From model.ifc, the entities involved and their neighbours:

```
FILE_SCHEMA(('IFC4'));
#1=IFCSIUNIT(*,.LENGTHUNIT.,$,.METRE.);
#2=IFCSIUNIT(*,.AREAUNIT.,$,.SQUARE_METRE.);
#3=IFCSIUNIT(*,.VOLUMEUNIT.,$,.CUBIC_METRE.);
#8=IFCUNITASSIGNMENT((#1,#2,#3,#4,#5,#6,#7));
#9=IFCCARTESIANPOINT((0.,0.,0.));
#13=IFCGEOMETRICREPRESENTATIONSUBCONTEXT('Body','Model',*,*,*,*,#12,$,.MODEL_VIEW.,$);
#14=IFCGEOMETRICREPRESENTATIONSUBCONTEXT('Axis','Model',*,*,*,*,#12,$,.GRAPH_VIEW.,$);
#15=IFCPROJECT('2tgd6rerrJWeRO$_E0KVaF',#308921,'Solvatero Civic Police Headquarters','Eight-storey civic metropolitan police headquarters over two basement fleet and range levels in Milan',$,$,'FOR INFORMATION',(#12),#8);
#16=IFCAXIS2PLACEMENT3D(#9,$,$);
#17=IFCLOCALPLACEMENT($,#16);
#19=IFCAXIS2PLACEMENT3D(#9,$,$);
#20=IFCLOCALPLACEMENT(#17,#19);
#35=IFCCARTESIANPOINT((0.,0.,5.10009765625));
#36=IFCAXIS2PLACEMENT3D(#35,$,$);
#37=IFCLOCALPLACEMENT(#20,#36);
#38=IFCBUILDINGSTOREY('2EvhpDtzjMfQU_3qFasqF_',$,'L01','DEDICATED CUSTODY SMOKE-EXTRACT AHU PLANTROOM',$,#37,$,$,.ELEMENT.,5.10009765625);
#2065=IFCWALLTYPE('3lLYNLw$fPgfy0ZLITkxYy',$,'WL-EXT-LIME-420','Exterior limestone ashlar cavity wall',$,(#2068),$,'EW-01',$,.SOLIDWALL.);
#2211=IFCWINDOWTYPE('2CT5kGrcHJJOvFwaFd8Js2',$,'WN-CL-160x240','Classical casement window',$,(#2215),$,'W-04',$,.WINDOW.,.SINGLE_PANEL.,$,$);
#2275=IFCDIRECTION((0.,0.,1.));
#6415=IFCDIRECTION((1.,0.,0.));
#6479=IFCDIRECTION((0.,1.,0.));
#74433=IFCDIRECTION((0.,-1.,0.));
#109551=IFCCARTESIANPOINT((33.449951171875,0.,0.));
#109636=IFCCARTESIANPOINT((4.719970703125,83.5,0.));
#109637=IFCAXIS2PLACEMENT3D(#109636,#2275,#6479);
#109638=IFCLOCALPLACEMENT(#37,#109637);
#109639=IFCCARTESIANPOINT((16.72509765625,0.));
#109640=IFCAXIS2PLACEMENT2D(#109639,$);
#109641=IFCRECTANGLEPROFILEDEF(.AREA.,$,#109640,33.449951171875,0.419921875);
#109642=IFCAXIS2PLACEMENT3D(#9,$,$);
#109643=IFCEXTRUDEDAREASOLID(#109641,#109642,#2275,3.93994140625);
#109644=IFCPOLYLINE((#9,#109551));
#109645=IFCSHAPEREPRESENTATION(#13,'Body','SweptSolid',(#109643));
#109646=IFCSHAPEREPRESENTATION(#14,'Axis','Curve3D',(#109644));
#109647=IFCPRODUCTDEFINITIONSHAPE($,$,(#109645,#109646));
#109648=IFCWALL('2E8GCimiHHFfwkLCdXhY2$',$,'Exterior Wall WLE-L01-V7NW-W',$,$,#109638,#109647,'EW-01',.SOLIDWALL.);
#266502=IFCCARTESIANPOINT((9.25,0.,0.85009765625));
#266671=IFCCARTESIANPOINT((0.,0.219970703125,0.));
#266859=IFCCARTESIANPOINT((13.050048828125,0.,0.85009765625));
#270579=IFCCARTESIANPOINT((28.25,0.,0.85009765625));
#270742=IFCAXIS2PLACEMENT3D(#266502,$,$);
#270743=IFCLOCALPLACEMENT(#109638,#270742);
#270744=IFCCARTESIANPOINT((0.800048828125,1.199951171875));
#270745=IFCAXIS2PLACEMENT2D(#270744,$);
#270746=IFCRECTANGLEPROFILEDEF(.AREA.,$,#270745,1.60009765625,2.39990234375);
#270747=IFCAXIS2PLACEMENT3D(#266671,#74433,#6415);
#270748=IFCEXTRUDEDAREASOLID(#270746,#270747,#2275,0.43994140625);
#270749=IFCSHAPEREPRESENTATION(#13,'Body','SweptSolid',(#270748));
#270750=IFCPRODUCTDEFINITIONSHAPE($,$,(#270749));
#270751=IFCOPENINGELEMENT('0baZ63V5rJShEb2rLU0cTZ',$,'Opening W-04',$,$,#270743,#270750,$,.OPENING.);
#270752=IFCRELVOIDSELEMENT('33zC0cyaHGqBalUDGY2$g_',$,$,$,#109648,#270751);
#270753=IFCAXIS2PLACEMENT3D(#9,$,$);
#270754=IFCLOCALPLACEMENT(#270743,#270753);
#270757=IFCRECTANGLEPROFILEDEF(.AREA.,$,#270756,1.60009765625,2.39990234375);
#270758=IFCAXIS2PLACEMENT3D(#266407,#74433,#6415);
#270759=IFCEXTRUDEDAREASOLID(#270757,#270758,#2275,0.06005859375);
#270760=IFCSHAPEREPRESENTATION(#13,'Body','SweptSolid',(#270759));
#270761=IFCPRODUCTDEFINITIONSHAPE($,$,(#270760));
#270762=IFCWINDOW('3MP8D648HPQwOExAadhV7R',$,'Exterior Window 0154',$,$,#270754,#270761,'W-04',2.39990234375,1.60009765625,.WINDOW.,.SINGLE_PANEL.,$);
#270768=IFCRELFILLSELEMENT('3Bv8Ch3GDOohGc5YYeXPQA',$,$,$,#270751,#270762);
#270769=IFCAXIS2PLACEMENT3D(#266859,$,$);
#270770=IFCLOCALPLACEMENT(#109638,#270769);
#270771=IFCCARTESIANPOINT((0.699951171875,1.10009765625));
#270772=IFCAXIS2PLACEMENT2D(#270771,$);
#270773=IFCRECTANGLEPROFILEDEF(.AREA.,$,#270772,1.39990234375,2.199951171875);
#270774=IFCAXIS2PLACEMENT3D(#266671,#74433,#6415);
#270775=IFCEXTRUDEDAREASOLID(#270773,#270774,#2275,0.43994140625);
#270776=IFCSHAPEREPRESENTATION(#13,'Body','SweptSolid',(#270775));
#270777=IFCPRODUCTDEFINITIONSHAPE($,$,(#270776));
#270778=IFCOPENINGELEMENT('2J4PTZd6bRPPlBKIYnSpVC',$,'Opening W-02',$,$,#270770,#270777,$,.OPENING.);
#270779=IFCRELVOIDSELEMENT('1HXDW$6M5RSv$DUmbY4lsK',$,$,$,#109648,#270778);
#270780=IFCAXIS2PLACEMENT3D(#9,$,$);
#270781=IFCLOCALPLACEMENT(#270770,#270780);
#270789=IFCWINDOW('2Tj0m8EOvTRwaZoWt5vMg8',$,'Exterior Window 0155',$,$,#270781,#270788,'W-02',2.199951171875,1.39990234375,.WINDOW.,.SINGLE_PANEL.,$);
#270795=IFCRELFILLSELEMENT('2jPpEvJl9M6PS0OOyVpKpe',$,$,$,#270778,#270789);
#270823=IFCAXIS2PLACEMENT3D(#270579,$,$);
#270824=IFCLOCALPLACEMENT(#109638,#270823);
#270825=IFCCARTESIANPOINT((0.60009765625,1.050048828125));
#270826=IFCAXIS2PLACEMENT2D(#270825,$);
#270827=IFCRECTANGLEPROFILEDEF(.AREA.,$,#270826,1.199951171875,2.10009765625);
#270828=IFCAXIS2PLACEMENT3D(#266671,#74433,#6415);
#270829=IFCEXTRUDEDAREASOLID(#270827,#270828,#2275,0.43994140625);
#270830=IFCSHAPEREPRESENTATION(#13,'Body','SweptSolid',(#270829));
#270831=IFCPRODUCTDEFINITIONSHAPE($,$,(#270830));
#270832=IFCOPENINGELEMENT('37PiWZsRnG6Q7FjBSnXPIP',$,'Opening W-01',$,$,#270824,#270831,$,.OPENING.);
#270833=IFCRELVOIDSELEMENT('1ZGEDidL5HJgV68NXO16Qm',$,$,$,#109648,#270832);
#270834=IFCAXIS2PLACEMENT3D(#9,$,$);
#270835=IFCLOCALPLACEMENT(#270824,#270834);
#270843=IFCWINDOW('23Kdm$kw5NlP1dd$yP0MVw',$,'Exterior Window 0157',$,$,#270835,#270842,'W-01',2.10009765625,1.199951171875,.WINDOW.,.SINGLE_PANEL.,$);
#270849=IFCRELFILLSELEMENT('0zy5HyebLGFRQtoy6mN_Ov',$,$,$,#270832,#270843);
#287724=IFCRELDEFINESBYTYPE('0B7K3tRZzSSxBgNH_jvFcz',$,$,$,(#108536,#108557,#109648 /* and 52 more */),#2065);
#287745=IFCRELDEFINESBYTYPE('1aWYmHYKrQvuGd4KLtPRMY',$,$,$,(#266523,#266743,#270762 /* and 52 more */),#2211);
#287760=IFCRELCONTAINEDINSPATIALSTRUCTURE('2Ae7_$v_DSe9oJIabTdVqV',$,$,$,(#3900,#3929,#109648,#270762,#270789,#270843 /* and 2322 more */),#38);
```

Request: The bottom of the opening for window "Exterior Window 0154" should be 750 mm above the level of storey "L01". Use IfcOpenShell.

```python
import numpy as np
import ifcopenshell
import ifcopenshell.api.geometry
import ifcopenshell.geom
import ifcopenshell.util.element
import ifcopenshell.util.placement
import ifcopenshell.util.shape
import ifcopenshell.util.unit

model = ifcopenshell.open("model.ifc")
unit_scale = ifcopenshell.util.unit.calculate_unit_scale(model)

window = model.by_guid("3MP8D648HPQwOExAadhV7R")
opening = window.FillsVoids[0].RelatingOpeningElement
storey = ifcopenshell.util.element.get_container(window, ifc_class="IfcBuildingStorey")
level = ifcopenshell.util.placement.get_local_placement(storey.ObjectPlacement)[2, 3]

# The opening's origin need not be at the sill, so measure its lowest point.
shape = ifcopenshell.geom.create_shape(ifcopenshell.geom.settings(), opening)
bottom = ifcopenshell.util.shape.get_shape_bottom_elevation(shape, shape.geometry) / unit_scale
dz = level + 0.75 - bottom

shift = np.array([0.0, 0.0, dz])
# The window is placed relative to its opening, so it follows when the opening moves.
matrix = ifcopenshell.util.placement.get_local_placement(opening.ObjectPlacement)
matrix[:3, 3] += shift
ifcopenshell.api.geometry.edit_object_placement(
    model, product=opening, matrix=matrix, is_si=False, should_transform_children=True
)

print(f"moved by {dz * unit_scale:+.3f} m")

model.write("model_edited.ifc")
```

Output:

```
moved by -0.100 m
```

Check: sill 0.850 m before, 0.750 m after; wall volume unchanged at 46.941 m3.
